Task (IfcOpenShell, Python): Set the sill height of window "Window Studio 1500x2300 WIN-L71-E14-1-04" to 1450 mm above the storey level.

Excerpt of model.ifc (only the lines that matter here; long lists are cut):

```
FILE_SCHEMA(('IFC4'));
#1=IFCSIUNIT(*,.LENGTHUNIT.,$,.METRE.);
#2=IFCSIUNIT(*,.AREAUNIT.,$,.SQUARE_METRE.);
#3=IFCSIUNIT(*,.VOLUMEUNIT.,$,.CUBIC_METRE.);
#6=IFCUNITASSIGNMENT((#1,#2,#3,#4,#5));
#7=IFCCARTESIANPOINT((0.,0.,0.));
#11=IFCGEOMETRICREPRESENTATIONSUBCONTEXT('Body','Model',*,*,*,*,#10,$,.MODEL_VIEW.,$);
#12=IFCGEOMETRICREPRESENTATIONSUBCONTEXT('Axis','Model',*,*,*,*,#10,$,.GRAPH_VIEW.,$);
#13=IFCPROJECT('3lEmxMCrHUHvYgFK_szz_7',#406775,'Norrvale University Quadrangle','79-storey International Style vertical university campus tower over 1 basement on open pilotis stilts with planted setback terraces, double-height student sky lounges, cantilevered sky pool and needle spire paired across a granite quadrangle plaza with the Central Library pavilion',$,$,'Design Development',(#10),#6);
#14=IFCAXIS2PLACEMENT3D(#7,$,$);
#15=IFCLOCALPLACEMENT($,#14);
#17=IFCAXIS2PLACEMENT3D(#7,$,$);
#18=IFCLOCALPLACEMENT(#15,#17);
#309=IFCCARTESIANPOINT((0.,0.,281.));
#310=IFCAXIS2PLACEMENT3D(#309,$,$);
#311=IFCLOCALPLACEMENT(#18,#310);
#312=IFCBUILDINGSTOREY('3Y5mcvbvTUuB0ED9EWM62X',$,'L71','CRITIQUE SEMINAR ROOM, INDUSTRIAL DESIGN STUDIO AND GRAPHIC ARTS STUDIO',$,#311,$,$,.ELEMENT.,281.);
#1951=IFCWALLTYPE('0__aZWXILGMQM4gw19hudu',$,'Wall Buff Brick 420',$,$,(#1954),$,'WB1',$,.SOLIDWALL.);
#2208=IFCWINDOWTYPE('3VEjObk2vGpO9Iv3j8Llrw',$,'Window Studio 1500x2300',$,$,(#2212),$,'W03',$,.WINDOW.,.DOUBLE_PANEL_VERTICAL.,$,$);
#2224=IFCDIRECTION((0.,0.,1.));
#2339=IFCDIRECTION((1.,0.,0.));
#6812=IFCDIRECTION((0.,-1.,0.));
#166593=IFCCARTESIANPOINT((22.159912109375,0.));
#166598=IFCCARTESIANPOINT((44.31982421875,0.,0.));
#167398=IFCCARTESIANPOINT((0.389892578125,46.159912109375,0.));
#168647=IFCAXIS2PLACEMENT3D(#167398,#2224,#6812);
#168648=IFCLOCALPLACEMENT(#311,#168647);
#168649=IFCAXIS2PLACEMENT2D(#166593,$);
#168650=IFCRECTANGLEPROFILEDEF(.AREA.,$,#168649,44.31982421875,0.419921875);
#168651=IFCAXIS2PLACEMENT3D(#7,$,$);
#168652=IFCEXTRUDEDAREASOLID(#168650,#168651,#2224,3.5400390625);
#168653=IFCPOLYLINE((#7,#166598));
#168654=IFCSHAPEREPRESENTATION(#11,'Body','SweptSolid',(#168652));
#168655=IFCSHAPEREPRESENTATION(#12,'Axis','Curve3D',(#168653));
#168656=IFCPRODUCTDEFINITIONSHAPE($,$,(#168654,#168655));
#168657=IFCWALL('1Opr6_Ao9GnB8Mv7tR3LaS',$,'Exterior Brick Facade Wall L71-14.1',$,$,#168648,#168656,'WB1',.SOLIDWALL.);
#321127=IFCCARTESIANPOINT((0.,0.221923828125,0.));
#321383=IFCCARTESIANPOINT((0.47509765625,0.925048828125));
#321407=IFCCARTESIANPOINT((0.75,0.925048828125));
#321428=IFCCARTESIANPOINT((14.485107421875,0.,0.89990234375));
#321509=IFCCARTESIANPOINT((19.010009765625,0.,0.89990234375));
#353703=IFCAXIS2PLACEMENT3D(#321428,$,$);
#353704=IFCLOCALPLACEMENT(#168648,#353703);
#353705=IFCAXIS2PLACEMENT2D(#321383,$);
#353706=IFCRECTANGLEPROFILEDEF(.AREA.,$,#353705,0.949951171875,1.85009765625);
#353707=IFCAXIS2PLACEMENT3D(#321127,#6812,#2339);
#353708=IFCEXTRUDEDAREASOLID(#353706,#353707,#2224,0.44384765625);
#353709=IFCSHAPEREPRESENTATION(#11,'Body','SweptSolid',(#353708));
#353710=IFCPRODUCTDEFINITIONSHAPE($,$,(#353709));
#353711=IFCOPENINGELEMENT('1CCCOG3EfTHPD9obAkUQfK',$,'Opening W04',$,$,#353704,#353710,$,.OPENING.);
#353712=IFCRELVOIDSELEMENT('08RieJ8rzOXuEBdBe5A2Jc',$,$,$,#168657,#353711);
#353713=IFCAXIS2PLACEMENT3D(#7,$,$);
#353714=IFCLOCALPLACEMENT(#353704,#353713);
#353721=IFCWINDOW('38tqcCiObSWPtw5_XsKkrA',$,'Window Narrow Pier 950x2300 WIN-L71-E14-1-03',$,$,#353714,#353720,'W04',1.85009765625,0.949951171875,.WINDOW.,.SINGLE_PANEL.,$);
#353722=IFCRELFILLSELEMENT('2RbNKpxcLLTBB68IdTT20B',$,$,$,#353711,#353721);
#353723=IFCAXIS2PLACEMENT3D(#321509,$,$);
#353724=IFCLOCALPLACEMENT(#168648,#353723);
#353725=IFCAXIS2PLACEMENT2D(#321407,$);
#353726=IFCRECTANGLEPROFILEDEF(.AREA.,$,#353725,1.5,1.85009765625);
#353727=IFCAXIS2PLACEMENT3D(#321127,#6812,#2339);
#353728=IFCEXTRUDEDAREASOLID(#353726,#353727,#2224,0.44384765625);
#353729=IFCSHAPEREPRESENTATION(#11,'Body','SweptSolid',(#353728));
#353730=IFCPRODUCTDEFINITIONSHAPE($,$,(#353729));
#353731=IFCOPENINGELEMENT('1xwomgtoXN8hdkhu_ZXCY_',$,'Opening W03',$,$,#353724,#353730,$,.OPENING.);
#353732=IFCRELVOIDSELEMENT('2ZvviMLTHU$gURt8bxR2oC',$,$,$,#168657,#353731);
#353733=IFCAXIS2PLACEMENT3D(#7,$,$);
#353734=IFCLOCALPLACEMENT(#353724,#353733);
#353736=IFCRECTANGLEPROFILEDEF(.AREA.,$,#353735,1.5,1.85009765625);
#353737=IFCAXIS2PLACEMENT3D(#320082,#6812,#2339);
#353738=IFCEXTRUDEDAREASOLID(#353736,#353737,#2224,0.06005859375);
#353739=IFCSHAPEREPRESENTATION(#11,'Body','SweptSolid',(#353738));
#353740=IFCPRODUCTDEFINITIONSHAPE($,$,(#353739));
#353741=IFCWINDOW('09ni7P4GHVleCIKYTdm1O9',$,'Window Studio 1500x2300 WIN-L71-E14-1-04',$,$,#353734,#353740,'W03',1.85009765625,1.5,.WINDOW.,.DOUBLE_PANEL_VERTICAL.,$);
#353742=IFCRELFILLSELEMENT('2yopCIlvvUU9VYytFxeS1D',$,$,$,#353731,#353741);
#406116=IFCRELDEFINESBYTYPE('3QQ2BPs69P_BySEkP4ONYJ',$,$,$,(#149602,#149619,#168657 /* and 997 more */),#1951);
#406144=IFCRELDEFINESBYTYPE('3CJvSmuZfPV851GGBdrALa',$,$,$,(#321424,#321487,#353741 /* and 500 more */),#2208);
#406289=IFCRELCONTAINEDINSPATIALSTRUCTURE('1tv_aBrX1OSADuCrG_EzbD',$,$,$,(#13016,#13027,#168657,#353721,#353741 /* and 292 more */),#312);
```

```python
import numpy as np
import ifcopenshell
import ifcopenshell.api.geometry
import ifcopenshell.geom
import ifcopenshell.util.element
import ifcopenshell.util.placement
import ifcopenshell.util.shape
import ifcopenshell.util.unit

model = ifcopenshell.open("model.ifc")
unit_scale = ifcopenshell.util.unit.calculate_unit_scale(model)

window = model.by_guid("09ni7P4GHVleCIKYTdm1O9")
opening = window.FillsVoids[0].RelatingOpeningElement
storey = ifcopenshell.util.element.get_container(window, ifc_class="IfcBuildingStorey")
level = ifcopenshell.util.placement.get_local_placement(storey.ObjectPlacement)[2, 3]

# The opening's origin need not be at the sill, so measure its lowest point.
shape = ifcopenshell.geom.create_shape(ifcopenshell.geom.settings(), opening)
bottom = ifcopenshell.util.shape.get_shape_bottom_elevation(shape, shape.geometry) / unit_scale
dz = level + 1.45 / unit_scale - bottom

shift = np.array([0.0, 0.0, dz])
# The window is placed relative to its opening, so it follows when the opening moves.
matrix = ifcopenshell.util.placement.get_local_placement(opening.ObjectPlacement)
matrix[:3, 3] += shift
ifcopenshell.api.geometry.edit_object_placement(
    model, product=opening, matrix=matrix, is_si=False, should_transform_children=True
)

print(f"moved by {dz * unit_scale:+.3f} m")

model.write("model_edited.ifc")
```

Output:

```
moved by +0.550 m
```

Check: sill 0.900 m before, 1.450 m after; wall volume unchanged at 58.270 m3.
